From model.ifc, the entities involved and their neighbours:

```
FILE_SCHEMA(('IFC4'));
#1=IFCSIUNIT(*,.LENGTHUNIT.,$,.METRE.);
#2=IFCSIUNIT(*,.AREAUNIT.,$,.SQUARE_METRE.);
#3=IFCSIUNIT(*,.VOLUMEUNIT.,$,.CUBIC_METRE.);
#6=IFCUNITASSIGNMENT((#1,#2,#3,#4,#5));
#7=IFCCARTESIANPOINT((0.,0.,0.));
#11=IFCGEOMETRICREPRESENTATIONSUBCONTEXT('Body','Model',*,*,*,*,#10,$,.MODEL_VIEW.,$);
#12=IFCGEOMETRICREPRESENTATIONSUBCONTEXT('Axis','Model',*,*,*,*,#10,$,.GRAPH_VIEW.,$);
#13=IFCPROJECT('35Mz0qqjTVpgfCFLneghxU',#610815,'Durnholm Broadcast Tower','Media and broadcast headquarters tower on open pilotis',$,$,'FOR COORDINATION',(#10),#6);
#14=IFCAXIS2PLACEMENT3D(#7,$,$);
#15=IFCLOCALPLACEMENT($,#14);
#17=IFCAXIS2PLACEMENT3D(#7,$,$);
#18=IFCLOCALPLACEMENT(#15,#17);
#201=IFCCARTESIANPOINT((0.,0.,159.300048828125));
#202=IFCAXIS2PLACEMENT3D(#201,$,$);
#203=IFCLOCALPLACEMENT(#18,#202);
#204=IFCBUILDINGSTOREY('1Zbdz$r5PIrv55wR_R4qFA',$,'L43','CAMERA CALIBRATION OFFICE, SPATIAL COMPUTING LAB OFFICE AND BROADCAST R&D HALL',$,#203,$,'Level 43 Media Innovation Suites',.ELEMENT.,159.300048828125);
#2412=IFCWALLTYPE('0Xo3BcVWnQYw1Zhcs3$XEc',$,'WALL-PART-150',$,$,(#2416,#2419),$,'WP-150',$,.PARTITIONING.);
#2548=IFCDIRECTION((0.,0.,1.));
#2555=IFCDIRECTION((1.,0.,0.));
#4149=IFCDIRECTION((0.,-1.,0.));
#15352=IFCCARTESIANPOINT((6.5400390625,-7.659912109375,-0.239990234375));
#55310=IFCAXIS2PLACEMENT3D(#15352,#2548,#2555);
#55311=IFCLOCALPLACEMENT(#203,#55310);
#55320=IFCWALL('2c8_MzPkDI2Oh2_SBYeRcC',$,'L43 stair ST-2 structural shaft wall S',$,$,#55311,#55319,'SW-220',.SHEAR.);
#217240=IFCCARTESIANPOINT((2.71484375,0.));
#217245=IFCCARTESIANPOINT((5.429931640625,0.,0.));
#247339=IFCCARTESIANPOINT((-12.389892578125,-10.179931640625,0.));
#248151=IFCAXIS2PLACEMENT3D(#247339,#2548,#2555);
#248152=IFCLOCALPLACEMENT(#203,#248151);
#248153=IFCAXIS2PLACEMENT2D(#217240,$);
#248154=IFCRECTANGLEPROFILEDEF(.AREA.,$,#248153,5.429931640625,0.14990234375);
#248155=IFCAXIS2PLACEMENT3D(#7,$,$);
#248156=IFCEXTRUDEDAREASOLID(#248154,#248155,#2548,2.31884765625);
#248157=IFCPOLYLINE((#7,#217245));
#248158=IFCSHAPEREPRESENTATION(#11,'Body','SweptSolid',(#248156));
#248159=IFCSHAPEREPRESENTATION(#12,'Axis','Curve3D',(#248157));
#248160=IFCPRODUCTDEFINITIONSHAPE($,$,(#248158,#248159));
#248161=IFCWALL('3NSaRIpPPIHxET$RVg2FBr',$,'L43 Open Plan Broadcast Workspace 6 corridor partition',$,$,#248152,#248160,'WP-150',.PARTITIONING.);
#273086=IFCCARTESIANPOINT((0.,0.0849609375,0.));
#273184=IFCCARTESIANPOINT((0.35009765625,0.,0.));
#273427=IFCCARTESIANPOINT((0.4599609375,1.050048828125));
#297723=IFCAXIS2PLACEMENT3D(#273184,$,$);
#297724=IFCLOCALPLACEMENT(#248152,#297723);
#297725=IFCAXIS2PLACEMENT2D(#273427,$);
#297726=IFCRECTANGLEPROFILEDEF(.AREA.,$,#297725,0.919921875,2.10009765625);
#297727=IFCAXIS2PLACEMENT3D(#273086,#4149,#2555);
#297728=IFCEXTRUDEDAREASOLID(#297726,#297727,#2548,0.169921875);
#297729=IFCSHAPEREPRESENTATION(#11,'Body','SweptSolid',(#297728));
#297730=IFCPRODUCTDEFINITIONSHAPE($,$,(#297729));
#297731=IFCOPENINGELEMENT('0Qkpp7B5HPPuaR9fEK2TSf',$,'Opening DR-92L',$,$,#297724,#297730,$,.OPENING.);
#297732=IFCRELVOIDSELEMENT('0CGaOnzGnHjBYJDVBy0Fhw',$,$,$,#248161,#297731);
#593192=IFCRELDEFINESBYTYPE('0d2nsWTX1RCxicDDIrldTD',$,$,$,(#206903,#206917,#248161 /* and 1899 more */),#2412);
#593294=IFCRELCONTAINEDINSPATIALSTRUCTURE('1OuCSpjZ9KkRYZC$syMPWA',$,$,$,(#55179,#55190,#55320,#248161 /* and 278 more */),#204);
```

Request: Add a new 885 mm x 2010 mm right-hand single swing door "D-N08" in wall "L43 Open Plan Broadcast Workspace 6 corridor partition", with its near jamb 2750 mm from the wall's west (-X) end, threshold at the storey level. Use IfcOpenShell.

```python
import numpy as np
import ifcopenshell
import ifcopenshell.api.feature
import ifcopenshell.api.geometry
import ifcopenshell.api.root
import ifcopenshell.api.spatial
import ifcopenshell.geom
import ifcopenshell.util.element
import ifcopenshell.util.placement
import ifcopenshell.util.representation
import ifcopenshell.util.shape
import ifcopenshell.util.unit

model = ifcopenshell.open("model.ifc")
unit_scale = ifcopenshell.util.unit.calculate_unit_scale(model)
settings = ifcopenshell.geom.settings()


def volume(element):
    """Net volume in cubic metres, openings subtracted."""
    shape = ifcopenshell.geom.create_shape(settings, element)
    return ifcopenshell.util.shape.get_volume(shape.geometry)


wall = model.by_guid("3NSaRIpPPIHxET$RVg2FBr")
storey = ifcopenshell.util.element.get_container(wall, ifc_class="IfcBuildingStorey")
context = ifcopenshell.util.representation.get_context(model, "Model", "Body", "MODEL_VIEW")
before = volume(wall)

width, height, from_end, sill = 0.885, 2.01, 2.75, 0.0  # metres

# The wall runs along its own X axis, and the end named is its -X end.
wall_shape = ifcopenshell.geom.create_shape(settings, wall)
x, y, z = ifcopenshell.util.shape.get_vertices(wall_shape.geometry).T
start = x.min() + from_end
face, thickness = float(y.min()), float(y.max() - y.min())
wall_matrix = ifcopenshell.util.placement.get_local_placement(wall.ObjectPlacement)
level = ifcopenshell.util.placement.get_local_placement(storey.ObjectPlacement)[2, 3]


def in_wall(x, y):
    """Placement at x, y metres in the wall's axes, at sill height."""
    matrix = wall_matrix.copy()
    matrix[:, 3] = wall_matrix @ np.array([x / unit_scale, y / unit_scale, 0.0, 1.0])
    matrix[2, 3] = level + sill / unit_scale
    return matrix


# Opening: a box that overshoots both wall faces by 50 mm.
opening = ifcopenshell.api.root.create_entity(model, ifc_class="IfcOpeningElement", predefined_type="OPENING")
box = ifcopenshell.api.geometry.add_wall_representation(
    model, context=context, length=width, height=height, thickness=thickness + 0.1
)
ifcopenshell.api.geometry.assign_representation(model, product=opening, representation=box)
ifcopenshell.api.geometry.edit_object_placement(model, product=opening, matrix=in_wall(start, face - 0.05), is_si=False)
ifcopenshell.api.feature.add_feature(model, feature=opening, element=wall)

door = ifcopenshell.api.root.create_entity(model, ifc_class="IfcDoor", name="D-N08", predefined_type="DOOR")
door.OverallWidth, door.OverallHeight = width / unit_scale, height / unit_scale
door.OperationType = "SINGLE_SWING_RIGHT"
body = ifcopenshell.api.geometry.add_door_representation(
    model,
    context=context,
    overall_width=door.OverallWidth,
    overall_height=door.OverallHeight,
    operation_type="SINGLE_SWING_RIGHT",
    lining_properties={"LiningDepth": thickness / unit_scale, "ThresholdDepth": thickness / unit_scale},
)
ifcopenshell.api.geometry.assign_representation(model, product=door, representation=body)
ifcopenshell.api.spatial.assign_container(model, products=[door], relating_structure=storey)
ifcopenshell.api.feature.add_filling(model, opening=opening, element=door)

# The lining spans the wall, so the door starts at the wall face.
ifcopenshell.api.geometry.edit_object_placement(model, product=door, matrix=in_wall(start, face), is_si=False)

after = volume(wall)

print(f"wall volume {before:.3f} -> {after:.3f} m3")

model.write("model_updated.ifc")
```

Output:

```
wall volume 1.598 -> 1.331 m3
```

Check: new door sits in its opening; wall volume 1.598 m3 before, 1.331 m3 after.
